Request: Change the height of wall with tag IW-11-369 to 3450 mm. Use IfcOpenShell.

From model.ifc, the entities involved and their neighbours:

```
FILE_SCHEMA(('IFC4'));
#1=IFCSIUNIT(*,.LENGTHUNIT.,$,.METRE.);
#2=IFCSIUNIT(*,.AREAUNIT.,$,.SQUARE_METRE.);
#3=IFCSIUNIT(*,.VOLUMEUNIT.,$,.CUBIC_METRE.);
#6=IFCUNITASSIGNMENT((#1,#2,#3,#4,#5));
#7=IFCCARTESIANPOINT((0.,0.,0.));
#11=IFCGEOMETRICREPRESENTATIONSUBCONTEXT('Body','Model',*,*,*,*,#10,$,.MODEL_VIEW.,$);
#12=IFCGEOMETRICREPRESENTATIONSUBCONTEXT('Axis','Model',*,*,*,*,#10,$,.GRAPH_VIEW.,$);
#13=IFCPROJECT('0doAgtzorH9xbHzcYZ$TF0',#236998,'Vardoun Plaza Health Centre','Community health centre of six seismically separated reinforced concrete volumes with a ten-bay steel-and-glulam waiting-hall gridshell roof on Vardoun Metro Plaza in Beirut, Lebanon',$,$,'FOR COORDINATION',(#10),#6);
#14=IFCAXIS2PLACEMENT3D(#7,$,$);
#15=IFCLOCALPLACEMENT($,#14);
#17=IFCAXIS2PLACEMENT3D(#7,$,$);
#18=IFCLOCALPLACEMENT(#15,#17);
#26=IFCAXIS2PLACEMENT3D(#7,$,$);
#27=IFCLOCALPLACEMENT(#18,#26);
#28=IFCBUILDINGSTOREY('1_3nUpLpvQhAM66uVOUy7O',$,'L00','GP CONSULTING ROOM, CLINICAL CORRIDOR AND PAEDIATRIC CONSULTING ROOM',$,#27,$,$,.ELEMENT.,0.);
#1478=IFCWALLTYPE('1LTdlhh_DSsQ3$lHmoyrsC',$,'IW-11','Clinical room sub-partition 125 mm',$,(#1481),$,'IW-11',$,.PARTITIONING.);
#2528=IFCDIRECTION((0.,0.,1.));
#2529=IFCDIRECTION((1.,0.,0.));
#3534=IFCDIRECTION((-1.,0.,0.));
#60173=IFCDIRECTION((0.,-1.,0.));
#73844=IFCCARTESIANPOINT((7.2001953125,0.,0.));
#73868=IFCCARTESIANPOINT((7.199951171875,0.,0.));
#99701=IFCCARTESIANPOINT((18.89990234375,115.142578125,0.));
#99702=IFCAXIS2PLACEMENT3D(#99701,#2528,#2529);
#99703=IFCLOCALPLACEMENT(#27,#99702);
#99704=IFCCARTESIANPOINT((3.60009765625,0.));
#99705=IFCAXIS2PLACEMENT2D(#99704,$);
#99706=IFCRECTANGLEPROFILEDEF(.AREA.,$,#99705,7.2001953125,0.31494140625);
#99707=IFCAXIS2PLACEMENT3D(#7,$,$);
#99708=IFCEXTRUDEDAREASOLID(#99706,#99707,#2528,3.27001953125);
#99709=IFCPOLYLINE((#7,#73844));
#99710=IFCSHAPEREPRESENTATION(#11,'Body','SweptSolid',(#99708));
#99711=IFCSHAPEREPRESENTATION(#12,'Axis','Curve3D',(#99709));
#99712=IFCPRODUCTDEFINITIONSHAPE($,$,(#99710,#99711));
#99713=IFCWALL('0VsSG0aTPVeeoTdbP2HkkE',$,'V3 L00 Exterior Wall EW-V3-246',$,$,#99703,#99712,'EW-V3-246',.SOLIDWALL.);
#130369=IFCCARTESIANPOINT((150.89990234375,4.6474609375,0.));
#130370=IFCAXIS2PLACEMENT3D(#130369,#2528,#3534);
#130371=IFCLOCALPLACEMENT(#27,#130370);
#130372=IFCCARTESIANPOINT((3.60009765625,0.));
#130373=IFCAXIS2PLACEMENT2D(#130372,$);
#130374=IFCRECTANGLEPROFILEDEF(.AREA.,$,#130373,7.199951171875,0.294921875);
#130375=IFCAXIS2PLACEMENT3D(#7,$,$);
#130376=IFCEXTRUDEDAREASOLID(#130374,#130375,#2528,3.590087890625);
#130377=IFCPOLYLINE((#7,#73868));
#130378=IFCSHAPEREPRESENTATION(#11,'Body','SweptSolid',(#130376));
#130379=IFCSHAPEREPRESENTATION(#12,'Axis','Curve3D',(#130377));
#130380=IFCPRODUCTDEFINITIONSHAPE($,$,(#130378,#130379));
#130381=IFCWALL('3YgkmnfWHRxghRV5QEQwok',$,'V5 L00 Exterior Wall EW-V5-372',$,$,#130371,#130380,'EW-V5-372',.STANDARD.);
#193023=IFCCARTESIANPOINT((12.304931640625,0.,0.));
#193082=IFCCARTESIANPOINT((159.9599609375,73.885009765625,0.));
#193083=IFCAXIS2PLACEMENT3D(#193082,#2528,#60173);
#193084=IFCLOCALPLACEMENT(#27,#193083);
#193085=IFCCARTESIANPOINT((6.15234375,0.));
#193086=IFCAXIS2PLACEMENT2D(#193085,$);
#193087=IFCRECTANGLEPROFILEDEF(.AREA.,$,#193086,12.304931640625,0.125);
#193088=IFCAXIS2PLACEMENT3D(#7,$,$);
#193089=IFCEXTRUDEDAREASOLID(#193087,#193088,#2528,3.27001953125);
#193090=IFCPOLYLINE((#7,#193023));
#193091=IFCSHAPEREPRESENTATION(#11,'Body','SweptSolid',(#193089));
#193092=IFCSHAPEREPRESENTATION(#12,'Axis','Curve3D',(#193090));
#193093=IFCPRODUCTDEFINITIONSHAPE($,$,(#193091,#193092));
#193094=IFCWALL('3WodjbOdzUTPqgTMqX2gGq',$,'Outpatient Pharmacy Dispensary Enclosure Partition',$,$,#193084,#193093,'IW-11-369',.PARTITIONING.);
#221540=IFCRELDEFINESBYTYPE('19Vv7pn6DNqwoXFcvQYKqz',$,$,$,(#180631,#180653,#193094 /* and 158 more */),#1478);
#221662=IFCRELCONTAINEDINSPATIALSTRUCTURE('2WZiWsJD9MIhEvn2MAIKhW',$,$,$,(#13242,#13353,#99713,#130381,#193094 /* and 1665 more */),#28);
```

```python
import ifcopenshell
import ifcopenshell.geom
import ifcopenshell.util.representation
import ifcopenshell.util.shape
import ifcopenshell.util.unit

model = ifcopenshell.open("model.ifc")
unit_scale = ifcopenshell.util.unit.calculate_unit_scale(model)
settings = ifcopenshell.geom.settings()


def volume(element):
    """Net volume in cubic metres, openings subtracted."""
    shape = ifcopenshell.geom.create_shape(settings, element)
    return ifcopenshell.util.shape.get_volume(shape.geometry)


wall = model.by_id(193094)
before = volume(wall)

body = ifcopenshell.util.representation.get_representation(wall, "Model", "Body")
solid = body.Items[0]
old_height = solid.Depth
solid.Depth = 3.45 / unit_scale
after = volume(wall)

print(f"height {old_height:g} -> {solid.Depth:g}, volume {before:.3f} -> {after:.3f} m3")

model.write("model_v2.ifc")
```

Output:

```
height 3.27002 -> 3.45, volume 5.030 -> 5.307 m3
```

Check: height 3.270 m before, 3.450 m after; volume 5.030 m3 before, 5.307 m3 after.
